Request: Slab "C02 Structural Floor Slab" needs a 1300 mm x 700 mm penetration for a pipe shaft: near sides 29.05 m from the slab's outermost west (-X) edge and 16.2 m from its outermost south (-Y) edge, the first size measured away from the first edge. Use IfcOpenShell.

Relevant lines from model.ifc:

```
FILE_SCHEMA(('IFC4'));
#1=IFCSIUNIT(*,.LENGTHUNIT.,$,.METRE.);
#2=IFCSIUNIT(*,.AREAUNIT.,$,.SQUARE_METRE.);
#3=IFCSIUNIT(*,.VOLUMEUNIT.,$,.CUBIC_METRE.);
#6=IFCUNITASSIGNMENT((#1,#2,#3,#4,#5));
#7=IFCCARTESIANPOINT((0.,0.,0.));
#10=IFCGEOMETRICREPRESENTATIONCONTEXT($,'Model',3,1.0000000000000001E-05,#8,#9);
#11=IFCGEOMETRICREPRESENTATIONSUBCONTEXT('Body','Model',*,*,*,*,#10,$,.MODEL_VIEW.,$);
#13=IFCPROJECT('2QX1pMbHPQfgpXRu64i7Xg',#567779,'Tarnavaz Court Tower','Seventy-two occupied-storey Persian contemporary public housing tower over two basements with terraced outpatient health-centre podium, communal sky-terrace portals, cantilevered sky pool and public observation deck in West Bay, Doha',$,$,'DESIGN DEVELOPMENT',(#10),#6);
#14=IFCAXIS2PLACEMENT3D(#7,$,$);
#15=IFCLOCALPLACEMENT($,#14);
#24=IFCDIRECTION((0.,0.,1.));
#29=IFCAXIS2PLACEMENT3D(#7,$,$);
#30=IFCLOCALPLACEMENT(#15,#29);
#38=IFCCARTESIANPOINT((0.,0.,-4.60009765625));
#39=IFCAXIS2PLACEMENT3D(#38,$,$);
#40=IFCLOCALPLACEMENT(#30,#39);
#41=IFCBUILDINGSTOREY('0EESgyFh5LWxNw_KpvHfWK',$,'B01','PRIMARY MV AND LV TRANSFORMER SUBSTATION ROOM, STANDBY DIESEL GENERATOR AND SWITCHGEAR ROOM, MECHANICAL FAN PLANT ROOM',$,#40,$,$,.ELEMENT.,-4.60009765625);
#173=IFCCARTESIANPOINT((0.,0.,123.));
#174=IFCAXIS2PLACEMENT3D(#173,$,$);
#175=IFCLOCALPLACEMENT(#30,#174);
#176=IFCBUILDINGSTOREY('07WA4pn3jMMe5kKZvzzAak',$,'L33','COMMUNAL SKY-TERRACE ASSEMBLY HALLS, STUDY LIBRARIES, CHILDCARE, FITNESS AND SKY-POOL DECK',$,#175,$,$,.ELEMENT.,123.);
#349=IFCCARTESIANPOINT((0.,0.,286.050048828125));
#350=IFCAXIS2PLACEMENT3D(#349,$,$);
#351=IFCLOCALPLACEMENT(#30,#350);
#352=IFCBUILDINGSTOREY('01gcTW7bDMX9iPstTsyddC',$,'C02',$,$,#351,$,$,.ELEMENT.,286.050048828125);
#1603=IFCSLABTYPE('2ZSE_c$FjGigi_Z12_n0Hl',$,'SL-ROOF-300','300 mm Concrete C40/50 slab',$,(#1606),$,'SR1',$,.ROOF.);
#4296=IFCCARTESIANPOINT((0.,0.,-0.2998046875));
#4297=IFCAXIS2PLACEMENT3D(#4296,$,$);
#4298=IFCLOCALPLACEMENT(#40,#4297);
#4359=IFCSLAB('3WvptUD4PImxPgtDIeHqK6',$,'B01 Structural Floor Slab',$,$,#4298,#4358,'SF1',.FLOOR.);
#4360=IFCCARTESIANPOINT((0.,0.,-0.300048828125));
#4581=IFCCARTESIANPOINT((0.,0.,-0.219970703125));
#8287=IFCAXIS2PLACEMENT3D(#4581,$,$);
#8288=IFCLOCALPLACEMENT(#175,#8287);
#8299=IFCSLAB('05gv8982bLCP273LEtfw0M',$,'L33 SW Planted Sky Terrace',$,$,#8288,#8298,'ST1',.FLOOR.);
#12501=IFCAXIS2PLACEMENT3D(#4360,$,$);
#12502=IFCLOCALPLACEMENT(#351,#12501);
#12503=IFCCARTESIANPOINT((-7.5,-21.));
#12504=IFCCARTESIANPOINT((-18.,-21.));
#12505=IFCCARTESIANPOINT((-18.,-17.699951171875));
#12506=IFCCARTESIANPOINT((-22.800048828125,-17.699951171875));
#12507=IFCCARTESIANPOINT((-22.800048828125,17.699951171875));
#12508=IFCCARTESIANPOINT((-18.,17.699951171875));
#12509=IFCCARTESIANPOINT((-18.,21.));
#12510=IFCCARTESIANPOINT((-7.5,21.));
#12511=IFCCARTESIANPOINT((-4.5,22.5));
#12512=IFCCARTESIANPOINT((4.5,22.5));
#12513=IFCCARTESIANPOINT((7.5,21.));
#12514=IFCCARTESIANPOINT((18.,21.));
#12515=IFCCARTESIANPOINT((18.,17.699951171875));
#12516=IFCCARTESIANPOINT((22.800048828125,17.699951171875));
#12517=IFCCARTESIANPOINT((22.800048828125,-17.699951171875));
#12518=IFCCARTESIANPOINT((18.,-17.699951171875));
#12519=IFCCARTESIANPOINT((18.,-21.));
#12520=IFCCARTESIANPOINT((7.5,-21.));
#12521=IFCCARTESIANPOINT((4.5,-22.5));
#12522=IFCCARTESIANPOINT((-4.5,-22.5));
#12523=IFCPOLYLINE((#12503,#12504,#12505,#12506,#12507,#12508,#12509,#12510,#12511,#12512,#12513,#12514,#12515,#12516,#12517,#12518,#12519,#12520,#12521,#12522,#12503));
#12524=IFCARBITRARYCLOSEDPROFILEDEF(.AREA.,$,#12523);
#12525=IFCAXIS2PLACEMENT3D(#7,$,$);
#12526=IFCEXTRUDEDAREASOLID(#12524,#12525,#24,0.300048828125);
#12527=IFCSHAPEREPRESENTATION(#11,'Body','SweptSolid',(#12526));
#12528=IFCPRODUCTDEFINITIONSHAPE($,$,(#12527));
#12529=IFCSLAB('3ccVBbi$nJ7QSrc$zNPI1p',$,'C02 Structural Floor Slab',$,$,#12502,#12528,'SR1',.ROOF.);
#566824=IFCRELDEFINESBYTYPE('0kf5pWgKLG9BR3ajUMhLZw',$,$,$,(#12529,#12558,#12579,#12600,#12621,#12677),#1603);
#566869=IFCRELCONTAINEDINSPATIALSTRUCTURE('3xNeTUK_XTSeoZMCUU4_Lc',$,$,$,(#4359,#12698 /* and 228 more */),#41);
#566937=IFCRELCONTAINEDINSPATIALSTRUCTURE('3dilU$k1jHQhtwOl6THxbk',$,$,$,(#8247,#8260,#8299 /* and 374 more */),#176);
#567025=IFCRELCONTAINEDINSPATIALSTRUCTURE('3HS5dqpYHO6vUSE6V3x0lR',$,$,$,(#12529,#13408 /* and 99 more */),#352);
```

```python
import numpy as np
import ifcopenshell
import ifcopenshell.api.feature
import ifcopenshell.api.geometry
import ifcopenshell.api.root
import ifcopenshell.geom
import ifcopenshell.util.placement
import ifcopenshell.util.representation
import ifcopenshell.util.shape
import ifcopenshell.util.unit

model = ifcopenshell.open("model.ifc")
unit_scale = ifcopenshell.util.unit.calculate_unit_scale(model)
settings = ifcopenshell.geom.settings()


def volume(element):
    """Net volume in cubic metres, openings subtracted."""
    shape = ifcopenshell.geom.create_shape(settings, element)
    return ifcopenshell.util.shape.get_volume(shape.geometry)


slab = model.by_guid("3ccVBbi$nJ7QSrc$zNPI1p")
before = volume(slab)

# Extent in the slab's own axes, in metres. The edges named are its -X and -Y sides.
slab_shape = ifcopenshell.geom.create_shape(settings, slab)
vertices = ifcopenshell.util.shape.get_vertices(slab_shape.geometry)
x_min, y_min, bottom = vertices.min(axis=0)
top = vertices[:, 2].max()

opening = ifcopenshell.api.root.create_entity(model, ifc_class="IfcOpeningElement", name="Pipe shaft opening", predefined_type="OPENING")
context = ifcopenshell.util.representation.get_context(model, "Model", "Body", "MODEL_VIEW")
width, depth = 1.3, 0.7
outline = [(0.0, 0.0), (width, 0.0), (width, depth), (0.0, depth), (0.0, 0.0)]
# Overshoot both faces by 50 mm so the cut is clean.
shape = ifcopenshell.api.geometry.add_slab_representation(
    model, context=context, depth=top - bottom + 0.1, polyline=outline
)
ifcopenshell.api.geometry.assign_representation(model, product=opening, representation=shape)

matrix = ifcopenshell.util.placement.get_local_placement(slab.ObjectPlacement)
matrix[:, 3] = matrix @ np.append(np.array([x_min + 29.05, y_min + 16.2, bottom - 0.05]) / unit_scale, 1.0)
ifcopenshell.api.geometry.edit_object_placement(model, product=opening, matrix=matrix, is_si=False)
ifcopenshell.api.feature.add_feature(model, feature=opening, element=slab)

after = volume(slab)

print(f"slab volume {before:.3f} -> {after:.3f} m3")

model.write("model_v2.ifc")
```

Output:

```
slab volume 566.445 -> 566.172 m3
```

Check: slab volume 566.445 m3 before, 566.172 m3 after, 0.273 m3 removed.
